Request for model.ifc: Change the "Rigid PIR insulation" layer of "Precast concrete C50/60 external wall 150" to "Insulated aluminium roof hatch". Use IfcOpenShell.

First a look at what the model holds.

```python
import ifcopenshell
import ifcopenshell.util.element

model = ifcopenshell.open("model.ifc")
print(model.schema)
for layer_set in model.by_type("IfcMaterialLayerSet"):
    if layer_set.LayerSetName == "Precast concrete C50/60 external wall 150":
        for layer in layer_set.MaterialLayers:
            print(layer.id(), layer.Material and layer.Material.Name, layer.LayerThickness, sep=" | ")
        print(len(ifcopenshell.util.element.get_elements_by_material(model, layer_set)), "elements and types use it")
print(sorted(m.Name for m in model.by_type("IfcMaterial") if m.Name)[:60])
```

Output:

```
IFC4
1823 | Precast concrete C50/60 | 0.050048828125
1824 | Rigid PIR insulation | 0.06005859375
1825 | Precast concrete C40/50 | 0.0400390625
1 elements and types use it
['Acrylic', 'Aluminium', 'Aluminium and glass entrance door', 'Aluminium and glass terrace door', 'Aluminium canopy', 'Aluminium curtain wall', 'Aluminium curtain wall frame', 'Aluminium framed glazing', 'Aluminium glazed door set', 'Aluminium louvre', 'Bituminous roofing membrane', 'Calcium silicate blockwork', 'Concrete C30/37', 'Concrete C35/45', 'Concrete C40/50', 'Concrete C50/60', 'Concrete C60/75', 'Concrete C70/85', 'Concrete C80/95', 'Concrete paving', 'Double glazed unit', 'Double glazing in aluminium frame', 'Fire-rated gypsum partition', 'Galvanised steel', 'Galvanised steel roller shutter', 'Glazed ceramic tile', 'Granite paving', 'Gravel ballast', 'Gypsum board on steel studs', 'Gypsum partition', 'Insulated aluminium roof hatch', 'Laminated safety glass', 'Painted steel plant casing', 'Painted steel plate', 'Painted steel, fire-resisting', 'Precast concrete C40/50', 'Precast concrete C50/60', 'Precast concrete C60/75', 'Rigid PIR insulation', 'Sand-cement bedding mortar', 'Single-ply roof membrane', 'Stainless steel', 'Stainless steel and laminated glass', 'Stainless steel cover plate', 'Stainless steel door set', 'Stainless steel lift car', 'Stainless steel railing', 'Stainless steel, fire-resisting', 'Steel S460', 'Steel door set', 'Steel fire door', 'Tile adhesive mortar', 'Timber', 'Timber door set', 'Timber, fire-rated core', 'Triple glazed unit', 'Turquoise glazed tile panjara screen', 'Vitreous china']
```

```python
import ifcopenshell
import ifcopenshell.api.material

model = ifcopenshell.open("model.ifc")

layer_set = next(s for s in model.by_type("IfcMaterialLayerSet") if s.LayerSetName == "Precast concrete C50/60 external wall 150")
layer = next(l for l in layer_set.MaterialLayers if l.Material and l.Material.Name == "Rigid PIR insulation")
material = next(m for m in model.by_type("IfcMaterial") if m.Name == "Insulated aluminium roof hatch")

# Point this one layer at the other material; renaming the old one would change it everywhere.
ifcopenshell.api.material.edit_layer(model, layer=layer, attributes={}, material=material)

print([l.Material.Name if l.Material else None for l in layer_set.MaterialLayers])

model.write("model_v2.ifc")
```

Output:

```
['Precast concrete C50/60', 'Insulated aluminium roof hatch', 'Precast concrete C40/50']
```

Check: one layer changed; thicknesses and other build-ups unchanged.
